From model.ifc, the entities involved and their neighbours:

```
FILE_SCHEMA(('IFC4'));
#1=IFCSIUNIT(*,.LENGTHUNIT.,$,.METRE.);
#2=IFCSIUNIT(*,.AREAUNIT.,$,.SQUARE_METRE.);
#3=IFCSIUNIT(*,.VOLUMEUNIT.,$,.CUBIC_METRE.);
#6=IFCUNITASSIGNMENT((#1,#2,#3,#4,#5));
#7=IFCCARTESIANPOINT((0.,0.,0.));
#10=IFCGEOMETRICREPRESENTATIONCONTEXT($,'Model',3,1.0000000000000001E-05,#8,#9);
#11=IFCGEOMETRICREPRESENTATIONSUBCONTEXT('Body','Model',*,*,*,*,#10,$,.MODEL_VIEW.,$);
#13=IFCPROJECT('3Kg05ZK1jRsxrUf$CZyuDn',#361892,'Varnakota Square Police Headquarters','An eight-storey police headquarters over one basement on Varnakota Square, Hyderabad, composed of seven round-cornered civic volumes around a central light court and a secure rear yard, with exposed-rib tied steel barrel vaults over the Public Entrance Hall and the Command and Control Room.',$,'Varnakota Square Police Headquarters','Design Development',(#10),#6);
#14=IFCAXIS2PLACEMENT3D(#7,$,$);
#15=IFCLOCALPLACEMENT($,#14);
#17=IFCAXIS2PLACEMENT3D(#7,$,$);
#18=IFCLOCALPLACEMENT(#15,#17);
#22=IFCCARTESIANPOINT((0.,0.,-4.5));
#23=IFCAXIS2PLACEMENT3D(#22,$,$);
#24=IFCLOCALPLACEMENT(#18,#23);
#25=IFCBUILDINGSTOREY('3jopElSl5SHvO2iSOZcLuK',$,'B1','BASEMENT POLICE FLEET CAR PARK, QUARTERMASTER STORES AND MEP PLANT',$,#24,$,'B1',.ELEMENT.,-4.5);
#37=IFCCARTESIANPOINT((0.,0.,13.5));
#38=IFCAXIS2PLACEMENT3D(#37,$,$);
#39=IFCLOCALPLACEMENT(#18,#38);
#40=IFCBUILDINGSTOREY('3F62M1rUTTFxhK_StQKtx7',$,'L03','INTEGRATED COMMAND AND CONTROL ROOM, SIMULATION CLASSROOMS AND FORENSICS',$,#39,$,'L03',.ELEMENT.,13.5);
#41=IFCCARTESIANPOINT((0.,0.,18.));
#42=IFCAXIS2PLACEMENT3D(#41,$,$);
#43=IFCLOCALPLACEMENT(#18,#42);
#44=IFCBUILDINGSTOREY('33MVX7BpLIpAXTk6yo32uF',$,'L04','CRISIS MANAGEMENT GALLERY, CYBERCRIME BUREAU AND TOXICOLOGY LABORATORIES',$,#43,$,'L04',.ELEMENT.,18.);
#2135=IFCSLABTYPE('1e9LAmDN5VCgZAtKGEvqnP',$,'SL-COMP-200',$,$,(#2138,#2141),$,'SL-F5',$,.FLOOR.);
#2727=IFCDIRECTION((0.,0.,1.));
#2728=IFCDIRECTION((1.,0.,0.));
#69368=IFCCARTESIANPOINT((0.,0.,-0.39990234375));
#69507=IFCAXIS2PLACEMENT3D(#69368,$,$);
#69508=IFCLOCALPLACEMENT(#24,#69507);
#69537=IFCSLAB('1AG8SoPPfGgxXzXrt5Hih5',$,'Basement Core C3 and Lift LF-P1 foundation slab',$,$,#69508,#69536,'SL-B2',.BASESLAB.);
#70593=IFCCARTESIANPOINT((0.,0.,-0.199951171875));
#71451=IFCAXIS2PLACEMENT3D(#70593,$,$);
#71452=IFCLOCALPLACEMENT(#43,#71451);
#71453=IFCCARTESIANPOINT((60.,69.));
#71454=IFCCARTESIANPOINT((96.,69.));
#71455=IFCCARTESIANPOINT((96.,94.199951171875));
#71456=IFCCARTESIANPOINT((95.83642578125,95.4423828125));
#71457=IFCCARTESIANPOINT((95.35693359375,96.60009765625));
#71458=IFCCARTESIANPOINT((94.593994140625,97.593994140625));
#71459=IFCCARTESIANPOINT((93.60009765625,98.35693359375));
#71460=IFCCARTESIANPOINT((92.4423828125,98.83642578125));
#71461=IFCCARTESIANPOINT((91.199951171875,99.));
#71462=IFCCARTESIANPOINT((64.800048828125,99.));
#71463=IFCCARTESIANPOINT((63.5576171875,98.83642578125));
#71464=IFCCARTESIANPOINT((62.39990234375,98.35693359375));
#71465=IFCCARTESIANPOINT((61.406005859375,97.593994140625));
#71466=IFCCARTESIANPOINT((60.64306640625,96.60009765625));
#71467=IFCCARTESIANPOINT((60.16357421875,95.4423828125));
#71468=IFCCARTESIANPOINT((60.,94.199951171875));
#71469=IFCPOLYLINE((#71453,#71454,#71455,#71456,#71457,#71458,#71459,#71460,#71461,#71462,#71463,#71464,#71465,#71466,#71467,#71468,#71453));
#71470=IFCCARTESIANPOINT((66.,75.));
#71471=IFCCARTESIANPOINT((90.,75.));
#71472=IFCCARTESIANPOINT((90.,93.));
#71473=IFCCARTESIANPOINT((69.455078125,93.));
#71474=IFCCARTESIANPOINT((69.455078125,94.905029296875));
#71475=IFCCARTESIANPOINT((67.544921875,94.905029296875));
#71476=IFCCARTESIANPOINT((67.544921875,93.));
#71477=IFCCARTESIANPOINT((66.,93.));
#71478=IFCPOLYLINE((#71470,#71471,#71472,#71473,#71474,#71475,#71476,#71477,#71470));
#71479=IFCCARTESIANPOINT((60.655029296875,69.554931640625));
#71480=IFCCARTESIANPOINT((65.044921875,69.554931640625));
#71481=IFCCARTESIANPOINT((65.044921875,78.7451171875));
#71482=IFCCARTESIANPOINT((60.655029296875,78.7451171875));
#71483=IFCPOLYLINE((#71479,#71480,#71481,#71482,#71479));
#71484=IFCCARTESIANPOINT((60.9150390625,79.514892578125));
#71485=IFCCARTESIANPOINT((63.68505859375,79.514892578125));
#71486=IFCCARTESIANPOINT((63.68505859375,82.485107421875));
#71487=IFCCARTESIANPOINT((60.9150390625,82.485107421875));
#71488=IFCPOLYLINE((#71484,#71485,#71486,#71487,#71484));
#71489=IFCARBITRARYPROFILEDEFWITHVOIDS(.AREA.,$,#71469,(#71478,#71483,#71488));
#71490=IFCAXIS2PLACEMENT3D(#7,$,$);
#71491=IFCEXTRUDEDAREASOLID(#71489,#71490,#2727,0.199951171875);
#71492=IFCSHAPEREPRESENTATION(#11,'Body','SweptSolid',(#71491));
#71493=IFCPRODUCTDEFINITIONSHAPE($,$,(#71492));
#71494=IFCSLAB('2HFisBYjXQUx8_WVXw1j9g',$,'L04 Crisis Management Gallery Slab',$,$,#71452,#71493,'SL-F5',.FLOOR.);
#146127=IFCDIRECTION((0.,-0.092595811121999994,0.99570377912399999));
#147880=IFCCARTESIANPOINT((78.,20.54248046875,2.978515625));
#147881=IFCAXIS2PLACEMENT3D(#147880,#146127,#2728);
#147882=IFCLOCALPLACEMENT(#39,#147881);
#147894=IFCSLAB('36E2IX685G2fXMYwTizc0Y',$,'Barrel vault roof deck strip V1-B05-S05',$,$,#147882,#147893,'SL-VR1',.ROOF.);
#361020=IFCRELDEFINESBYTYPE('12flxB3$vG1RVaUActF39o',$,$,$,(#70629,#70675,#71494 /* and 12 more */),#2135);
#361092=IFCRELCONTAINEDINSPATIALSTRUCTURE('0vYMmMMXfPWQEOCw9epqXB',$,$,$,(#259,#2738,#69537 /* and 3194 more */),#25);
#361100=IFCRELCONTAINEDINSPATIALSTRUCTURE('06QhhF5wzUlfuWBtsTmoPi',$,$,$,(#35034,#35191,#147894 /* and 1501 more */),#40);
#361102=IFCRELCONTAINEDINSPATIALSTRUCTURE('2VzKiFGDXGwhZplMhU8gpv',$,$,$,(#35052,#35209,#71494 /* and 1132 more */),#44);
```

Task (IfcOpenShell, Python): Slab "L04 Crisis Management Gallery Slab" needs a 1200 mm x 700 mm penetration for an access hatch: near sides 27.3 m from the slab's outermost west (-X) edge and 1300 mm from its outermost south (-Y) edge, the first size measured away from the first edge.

```python
import numpy as np
import ifcopenshell
import ifcopenshell.api.feature
import ifcopenshell.api.geometry
import ifcopenshell.api.root
import ifcopenshell.geom
import ifcopenshell.util.placement
import ifcopenshell.util.representation
import ifcopenshell.util.shape
import ifcopenshell.util.unit

model = ifcopenshell.open("model.ifc")
unit_scale = ifcopenshell.util.unit.calculate_unit_scale(model)
settings = ifcopenshell.geom.settings()


def volume(element):
    """Net volume in cubic metres, openings subtracted."""
    shape = ifcopenshell.geom.create_shape(settings, element)
    return ifcopenshell.util.shape.get_volume(shape.geometry)


slab = model.by_id(71494)
before = volume(slab)

# Extent in the slab's own axes, in metres. The edges named are its -X and -Y sides.
slab_shape = ifcopenshell.geom.create_shape(settings, slab)
vertices = ifcopenshell.util.shape.get_vertices(slab_shape.geometry)
x_min, y_min, bottom = vertices.min(axis=0)
top = vertices[:, 2].max()

opening = ifcopenshell.api.root.create_entity(model, ifc_class="IfcOpeningElement", name="Access hatch opening", predefined_type="OPENING")
context = ifcopenshell.util.representation.get_context(model, "Model", "Body", "MODEL_VIEW")
width, depth = 1.2, 0.7
outline = [(0.0, 0.0), (width, 0.0), (width, depth), (0.0, depth), (0.0, 0.0)]
# Overshoot both faces by 50 mm so the cut is clean.
shape = ifcopenshell.api.geometry.add_slab_representation(
    model, context=context, depth=top - bottom + 0.1, polyline=outline
)
ifcopenshell.api.geometry.assign_representation(model, product=opening, representation=shape)

matrix = ifcopenshell.util.placement.get_local_placement(slab.ObjectPlacement)
matrix[:, 3] = matrix @ np.append(np.array([x_min + 27.3, y_min + 1.3, bottom - 0.05]) / unit_scale, 1.0)
ifcopenshell.api.geometry.edit_object_placement(model, product=opening, matrix=matrix, is_si=False)
ifcopenshell.api.feature.add_feature(model, feature=opening, element=slab)

after = volume(slab)

print(f"slab volume {before:.3f} -> {after:.3f} m3")

model.write("model-out.ifc")
```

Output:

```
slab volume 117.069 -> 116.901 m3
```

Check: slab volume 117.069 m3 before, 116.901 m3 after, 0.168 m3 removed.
